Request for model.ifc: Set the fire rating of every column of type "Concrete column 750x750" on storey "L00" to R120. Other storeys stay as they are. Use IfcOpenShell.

First a look at what the model holds.

```python
import ifcopenshell
import ifcopenshell.util.element

model = ifcopenshell.open("model.ifc")
print(model.schema)
storey = next(s for s in model.by_type("IfcBuildingStorey") if s.Name == "L00")
columns = [e for e in ifcopenshell.util.element.get_decomposition(storey) if e.is_a("IfcColumn")]
seen = {}
for e in columns:
    element_type = ifcopenshell.util.element.get_type(e)
    key = (element_type.Name if element_type != e and element_type else None, ifcopenshell.util.element.get_pset(e, "Pset_ColumnCommon", "FireRating"))
    seen[key] = seen.get(key, 0) + 1
for (name, value), count in sorted(seen.items(), key=str):
    print(count, "x", name, "|", value)
```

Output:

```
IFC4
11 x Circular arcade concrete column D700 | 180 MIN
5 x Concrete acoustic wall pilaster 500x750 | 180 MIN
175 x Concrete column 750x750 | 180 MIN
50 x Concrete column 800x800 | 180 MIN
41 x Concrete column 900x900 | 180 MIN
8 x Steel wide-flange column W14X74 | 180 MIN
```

```python
import ifcopenshell
import ifcopenshell.api.pset
import ifcopenshell.util.element

model = ifcopenshell.open("model.ifc")

storey = next(s for s in model.by_type("IfcBuildingStorey") if s.Name == "L00")
columns = [e for e in ifcopenshell.util.element.get_decomposition(storey) if e.is_a("IfcColumn")]

count = 0
for e in columns:
    element_type = ifcopenshell.util.element.get_type(e)
    if element_type in (None, e) or element_type.Name != "Concrete column 750x750":
        continue
    # add_pset returns the element's existing set when there is one.
    pset = ifcopenshell.api.pset.add_pset(model, product=e, name="Pset_ColumnCommon")
    ifcopenshell.api.pset.edit_pset(model, pset=pset, properties={"FireRating": "R120"})
    count += 1

print(count, "columns updated")

model.write("model_updated.ifc")
```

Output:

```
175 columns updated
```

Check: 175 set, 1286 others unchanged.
